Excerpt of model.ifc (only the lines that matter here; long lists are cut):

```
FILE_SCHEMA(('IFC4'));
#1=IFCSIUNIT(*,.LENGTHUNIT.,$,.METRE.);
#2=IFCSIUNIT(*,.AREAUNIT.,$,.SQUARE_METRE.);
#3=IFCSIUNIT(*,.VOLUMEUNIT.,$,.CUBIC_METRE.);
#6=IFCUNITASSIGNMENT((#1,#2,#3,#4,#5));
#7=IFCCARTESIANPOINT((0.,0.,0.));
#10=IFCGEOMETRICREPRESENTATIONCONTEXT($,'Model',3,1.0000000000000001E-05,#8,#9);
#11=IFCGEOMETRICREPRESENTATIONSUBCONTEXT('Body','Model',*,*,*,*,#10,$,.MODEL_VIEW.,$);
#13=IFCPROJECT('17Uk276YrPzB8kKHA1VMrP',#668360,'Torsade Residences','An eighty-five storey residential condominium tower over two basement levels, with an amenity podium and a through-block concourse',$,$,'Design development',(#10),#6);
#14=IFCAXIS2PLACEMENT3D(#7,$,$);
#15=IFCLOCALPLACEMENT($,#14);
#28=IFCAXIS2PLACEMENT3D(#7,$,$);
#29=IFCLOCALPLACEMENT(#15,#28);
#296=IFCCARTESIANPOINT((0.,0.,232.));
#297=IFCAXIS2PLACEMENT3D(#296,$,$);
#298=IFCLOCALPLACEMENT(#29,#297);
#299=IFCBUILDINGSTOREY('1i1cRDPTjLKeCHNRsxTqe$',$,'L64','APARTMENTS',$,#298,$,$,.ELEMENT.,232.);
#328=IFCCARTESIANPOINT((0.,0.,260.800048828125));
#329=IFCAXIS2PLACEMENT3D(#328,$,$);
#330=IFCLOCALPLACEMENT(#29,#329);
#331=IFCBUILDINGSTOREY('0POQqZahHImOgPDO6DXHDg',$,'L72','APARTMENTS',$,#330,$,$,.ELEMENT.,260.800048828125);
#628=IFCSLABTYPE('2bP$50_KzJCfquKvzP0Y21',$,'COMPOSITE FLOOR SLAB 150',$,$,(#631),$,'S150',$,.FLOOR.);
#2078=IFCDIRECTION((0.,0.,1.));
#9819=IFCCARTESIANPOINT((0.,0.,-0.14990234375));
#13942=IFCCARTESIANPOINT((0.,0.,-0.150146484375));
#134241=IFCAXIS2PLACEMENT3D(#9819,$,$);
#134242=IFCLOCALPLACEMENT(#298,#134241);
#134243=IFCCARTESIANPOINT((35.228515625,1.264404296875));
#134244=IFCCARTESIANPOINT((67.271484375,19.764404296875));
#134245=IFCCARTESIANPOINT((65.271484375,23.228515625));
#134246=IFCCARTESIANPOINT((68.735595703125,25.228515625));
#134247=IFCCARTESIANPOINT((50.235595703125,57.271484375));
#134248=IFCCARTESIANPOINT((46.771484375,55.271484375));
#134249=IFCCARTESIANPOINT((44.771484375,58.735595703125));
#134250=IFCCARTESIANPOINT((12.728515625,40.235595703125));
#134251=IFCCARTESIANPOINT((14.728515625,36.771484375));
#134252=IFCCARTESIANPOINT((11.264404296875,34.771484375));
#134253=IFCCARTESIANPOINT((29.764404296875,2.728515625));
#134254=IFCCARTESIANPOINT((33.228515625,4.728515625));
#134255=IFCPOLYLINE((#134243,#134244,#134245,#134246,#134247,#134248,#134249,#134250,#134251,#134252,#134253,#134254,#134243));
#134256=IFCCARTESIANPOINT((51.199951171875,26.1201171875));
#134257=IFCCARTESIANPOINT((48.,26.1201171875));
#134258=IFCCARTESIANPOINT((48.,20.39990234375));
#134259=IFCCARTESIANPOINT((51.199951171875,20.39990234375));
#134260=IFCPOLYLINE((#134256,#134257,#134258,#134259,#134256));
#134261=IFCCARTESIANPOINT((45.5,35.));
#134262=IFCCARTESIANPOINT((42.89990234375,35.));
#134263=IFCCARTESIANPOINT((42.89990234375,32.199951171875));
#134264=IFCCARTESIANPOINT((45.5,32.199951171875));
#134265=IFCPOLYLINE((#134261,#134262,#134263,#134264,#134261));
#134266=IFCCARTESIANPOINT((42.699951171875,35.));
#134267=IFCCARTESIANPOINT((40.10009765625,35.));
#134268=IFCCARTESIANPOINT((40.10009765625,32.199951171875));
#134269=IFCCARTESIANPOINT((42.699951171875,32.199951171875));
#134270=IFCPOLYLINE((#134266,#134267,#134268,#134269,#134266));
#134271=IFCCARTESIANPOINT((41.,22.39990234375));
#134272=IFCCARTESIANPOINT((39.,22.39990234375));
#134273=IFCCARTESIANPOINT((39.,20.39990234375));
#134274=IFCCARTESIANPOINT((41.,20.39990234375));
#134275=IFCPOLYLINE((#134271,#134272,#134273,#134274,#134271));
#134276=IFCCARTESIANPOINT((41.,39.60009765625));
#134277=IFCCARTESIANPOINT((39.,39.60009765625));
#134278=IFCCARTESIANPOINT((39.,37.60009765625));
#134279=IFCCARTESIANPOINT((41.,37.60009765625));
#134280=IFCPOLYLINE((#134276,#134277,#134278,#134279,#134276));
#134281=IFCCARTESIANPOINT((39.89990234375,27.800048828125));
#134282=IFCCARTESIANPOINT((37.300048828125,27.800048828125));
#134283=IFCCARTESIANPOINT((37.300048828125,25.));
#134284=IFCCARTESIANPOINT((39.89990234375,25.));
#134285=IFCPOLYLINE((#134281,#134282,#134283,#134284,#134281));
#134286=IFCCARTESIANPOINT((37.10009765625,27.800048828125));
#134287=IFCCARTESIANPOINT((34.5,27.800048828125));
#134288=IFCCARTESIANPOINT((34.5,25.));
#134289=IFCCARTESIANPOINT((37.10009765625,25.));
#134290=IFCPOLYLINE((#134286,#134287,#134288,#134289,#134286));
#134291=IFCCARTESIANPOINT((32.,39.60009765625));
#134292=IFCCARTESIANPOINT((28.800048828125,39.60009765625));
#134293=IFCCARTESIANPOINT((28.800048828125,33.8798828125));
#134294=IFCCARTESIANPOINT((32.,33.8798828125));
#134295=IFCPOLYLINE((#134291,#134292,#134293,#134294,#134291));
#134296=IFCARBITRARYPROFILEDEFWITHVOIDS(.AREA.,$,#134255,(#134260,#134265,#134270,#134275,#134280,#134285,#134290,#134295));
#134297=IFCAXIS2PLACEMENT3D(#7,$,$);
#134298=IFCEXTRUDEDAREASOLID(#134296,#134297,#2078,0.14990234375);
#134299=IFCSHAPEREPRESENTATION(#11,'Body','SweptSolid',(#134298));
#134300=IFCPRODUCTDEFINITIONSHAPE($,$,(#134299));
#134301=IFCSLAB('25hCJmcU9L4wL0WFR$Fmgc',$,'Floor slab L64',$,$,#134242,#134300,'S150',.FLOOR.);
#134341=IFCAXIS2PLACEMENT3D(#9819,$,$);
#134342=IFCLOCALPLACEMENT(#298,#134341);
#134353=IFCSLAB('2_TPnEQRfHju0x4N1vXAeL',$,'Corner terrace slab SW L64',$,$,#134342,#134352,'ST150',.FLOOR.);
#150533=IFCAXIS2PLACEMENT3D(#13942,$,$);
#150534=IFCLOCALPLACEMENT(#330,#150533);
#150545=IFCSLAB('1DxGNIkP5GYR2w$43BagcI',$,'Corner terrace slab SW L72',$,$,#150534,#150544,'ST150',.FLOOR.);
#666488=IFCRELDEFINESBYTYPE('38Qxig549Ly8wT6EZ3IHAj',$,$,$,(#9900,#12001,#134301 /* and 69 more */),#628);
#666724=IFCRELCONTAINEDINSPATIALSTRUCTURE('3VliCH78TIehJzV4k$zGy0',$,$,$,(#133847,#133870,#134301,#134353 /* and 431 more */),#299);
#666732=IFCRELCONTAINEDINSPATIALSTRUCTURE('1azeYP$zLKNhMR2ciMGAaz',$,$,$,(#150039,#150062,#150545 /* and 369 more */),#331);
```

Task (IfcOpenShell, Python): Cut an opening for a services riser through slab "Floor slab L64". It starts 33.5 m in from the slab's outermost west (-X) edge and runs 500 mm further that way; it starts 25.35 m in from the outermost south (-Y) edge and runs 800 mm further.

```python
import numpy as np
import ifcopenshell
import ifcopenshell.api.feature
import ifcopenshell.api.geometry
import ifcopenshell.api.root
import ifcopenshell.geom
import ifcopenshell.util.placement
import ifcopenshell.util.representation
import ifcopenshell.util.shape
import ifcopenshell.util.unit

model = ifcopenshell.open("model.ifc")
unit_scale = ifcopenshell.util.unit.calculate_unit_scale(model)
settings = ifcopenshell.geom.settings()


def volume(element):
    """Net volume in cubic metres, openings subtracted."""
    shape = ifcopenshell.geom.create_shape(settings, element)
    return ifcopenshell.util.shape.get_volume(shape.geometry)


slab = model.by_guid("25hCJmcU9L4wL0WFR$Fmgc")
before = volume(slab)

# Extent in the slab's own axes, in metres. The edges named are its -X and -Y sides.
slab_shape = ifcopenshell.geom.create_shape(settings, slab)
vertices = ifcopenshell.util.shape.get_vertices(slab_shape.geometry)
x_min, y_min, bottom = vertices.min(axis=0)
top = vertices[:, 2].max()

opening = ifcopenshell.api.root.create_entity(model, ifc_class="IfcOpeningElement", name="Services riser opening", predefined_type="OPENING")
context = ifcopenshell.util.representation.get_context(model, "Model", "Body", "MODEL_VIEW")
width, depth = 0.5, 0.8
outline = [(0.0, 0.0), (width, 0.0), (width, depth), (0.0, depth), (0.0, 0.0)]
# Overshoot both faces by 50 mm so the cut is clean.
shape = ifcopenshell.api.geometry.add_slab_representation(
    model, context=context, depth=top - bottom + 0.1, polyline=outline
)
ifcopenshell.api.geometry.assign_representation(model, product=opening, representation=shape)

matrix = ifcopenshell.util.placement.get_local_placement(slab.ObjectPlacement)
matrix[:, 3] = matrix @ np.append(np.array([x_min + 33.5, y_min + 25.35, bottom - 0.05]) / unit_scale, 1.0)
ifcopenshell.api.geometry.edit_object_placement(model, product=opening, matrix=matrix, is_si=False)
ifcopenshell.api.feature.add_feature(model, feature=opening, element=slab)

after = volume(slab)

print(f"slab volume {before:.3f} -> {after:.3f} m3")

model.write("model_rev.ifc")
```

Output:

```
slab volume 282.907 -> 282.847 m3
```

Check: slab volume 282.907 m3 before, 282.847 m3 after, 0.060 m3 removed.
